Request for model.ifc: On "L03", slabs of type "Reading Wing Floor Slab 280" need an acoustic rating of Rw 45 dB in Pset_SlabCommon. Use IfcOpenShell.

First a look at what the model holds.

```python
import ifcopenshell
import ifcopenshell.util.element

model = ifcopenshell.open("model.ifc")
print(model.schema)
storey = next(s for s in model.by_type("IfcBuildingStorey") if s.Name == "L03")
slabs = [e for e in ifcopenshell.util.element.get_decomposition(storey) if e.is_a("IfcSlab")]
seen = {}
for e in slabs:
    element_type = ifcopenshell.util.element.get_type(e)
    key = (element_type.Name if element_type != e and element_type else None, ifcopenshell.util.element.get_pset(e, "Pset_SlabCommon", "AcousticRating"))
    seen[key] = seen.get(key, 0) + 1
for (name, value), count in sorted(seen.items(), key=str):
    print(count, "x", name, "|", value)
```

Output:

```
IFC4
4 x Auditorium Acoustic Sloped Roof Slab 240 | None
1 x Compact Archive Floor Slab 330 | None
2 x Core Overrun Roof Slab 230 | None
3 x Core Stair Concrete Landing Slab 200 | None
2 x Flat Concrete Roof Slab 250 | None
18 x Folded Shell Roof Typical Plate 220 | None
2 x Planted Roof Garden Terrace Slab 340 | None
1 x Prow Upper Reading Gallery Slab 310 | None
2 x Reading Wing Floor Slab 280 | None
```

```python
import ifcopenshell
import ifcopenshell.api.pset
import ifcopenshell.util.element

model = ifcopenshell.open("model.ifc")

storey = next(s for s in model.by_type("IfcBuildingStorey") if s.Name == "L03")
slabs = [e for e in ifcopenshell.util.element.get_decomposition(storey) if e.is_a("IfcSlab")]

count = 0
for e in slabs:
    element_type = ifcopenshell.util.element.get_type(e)
    if element_type in (None, e) or element_type.Name != "Reading Wing Floor Slab 280":
        continue
    # add_pset returns the element's existing set when there is one.
    pset = ifcopenshell.api.pset.add_pset(model, product=e, name="Pset_SlabCommon")
    ifcopenshell.api.pset.edit_pset(model, pset=pset, properties={"AcousticRating": "Rw 45 dB"})
    count += 1

print(count, "slabs updated")

model.write("model_v2.ifc")
```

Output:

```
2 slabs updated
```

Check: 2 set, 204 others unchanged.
